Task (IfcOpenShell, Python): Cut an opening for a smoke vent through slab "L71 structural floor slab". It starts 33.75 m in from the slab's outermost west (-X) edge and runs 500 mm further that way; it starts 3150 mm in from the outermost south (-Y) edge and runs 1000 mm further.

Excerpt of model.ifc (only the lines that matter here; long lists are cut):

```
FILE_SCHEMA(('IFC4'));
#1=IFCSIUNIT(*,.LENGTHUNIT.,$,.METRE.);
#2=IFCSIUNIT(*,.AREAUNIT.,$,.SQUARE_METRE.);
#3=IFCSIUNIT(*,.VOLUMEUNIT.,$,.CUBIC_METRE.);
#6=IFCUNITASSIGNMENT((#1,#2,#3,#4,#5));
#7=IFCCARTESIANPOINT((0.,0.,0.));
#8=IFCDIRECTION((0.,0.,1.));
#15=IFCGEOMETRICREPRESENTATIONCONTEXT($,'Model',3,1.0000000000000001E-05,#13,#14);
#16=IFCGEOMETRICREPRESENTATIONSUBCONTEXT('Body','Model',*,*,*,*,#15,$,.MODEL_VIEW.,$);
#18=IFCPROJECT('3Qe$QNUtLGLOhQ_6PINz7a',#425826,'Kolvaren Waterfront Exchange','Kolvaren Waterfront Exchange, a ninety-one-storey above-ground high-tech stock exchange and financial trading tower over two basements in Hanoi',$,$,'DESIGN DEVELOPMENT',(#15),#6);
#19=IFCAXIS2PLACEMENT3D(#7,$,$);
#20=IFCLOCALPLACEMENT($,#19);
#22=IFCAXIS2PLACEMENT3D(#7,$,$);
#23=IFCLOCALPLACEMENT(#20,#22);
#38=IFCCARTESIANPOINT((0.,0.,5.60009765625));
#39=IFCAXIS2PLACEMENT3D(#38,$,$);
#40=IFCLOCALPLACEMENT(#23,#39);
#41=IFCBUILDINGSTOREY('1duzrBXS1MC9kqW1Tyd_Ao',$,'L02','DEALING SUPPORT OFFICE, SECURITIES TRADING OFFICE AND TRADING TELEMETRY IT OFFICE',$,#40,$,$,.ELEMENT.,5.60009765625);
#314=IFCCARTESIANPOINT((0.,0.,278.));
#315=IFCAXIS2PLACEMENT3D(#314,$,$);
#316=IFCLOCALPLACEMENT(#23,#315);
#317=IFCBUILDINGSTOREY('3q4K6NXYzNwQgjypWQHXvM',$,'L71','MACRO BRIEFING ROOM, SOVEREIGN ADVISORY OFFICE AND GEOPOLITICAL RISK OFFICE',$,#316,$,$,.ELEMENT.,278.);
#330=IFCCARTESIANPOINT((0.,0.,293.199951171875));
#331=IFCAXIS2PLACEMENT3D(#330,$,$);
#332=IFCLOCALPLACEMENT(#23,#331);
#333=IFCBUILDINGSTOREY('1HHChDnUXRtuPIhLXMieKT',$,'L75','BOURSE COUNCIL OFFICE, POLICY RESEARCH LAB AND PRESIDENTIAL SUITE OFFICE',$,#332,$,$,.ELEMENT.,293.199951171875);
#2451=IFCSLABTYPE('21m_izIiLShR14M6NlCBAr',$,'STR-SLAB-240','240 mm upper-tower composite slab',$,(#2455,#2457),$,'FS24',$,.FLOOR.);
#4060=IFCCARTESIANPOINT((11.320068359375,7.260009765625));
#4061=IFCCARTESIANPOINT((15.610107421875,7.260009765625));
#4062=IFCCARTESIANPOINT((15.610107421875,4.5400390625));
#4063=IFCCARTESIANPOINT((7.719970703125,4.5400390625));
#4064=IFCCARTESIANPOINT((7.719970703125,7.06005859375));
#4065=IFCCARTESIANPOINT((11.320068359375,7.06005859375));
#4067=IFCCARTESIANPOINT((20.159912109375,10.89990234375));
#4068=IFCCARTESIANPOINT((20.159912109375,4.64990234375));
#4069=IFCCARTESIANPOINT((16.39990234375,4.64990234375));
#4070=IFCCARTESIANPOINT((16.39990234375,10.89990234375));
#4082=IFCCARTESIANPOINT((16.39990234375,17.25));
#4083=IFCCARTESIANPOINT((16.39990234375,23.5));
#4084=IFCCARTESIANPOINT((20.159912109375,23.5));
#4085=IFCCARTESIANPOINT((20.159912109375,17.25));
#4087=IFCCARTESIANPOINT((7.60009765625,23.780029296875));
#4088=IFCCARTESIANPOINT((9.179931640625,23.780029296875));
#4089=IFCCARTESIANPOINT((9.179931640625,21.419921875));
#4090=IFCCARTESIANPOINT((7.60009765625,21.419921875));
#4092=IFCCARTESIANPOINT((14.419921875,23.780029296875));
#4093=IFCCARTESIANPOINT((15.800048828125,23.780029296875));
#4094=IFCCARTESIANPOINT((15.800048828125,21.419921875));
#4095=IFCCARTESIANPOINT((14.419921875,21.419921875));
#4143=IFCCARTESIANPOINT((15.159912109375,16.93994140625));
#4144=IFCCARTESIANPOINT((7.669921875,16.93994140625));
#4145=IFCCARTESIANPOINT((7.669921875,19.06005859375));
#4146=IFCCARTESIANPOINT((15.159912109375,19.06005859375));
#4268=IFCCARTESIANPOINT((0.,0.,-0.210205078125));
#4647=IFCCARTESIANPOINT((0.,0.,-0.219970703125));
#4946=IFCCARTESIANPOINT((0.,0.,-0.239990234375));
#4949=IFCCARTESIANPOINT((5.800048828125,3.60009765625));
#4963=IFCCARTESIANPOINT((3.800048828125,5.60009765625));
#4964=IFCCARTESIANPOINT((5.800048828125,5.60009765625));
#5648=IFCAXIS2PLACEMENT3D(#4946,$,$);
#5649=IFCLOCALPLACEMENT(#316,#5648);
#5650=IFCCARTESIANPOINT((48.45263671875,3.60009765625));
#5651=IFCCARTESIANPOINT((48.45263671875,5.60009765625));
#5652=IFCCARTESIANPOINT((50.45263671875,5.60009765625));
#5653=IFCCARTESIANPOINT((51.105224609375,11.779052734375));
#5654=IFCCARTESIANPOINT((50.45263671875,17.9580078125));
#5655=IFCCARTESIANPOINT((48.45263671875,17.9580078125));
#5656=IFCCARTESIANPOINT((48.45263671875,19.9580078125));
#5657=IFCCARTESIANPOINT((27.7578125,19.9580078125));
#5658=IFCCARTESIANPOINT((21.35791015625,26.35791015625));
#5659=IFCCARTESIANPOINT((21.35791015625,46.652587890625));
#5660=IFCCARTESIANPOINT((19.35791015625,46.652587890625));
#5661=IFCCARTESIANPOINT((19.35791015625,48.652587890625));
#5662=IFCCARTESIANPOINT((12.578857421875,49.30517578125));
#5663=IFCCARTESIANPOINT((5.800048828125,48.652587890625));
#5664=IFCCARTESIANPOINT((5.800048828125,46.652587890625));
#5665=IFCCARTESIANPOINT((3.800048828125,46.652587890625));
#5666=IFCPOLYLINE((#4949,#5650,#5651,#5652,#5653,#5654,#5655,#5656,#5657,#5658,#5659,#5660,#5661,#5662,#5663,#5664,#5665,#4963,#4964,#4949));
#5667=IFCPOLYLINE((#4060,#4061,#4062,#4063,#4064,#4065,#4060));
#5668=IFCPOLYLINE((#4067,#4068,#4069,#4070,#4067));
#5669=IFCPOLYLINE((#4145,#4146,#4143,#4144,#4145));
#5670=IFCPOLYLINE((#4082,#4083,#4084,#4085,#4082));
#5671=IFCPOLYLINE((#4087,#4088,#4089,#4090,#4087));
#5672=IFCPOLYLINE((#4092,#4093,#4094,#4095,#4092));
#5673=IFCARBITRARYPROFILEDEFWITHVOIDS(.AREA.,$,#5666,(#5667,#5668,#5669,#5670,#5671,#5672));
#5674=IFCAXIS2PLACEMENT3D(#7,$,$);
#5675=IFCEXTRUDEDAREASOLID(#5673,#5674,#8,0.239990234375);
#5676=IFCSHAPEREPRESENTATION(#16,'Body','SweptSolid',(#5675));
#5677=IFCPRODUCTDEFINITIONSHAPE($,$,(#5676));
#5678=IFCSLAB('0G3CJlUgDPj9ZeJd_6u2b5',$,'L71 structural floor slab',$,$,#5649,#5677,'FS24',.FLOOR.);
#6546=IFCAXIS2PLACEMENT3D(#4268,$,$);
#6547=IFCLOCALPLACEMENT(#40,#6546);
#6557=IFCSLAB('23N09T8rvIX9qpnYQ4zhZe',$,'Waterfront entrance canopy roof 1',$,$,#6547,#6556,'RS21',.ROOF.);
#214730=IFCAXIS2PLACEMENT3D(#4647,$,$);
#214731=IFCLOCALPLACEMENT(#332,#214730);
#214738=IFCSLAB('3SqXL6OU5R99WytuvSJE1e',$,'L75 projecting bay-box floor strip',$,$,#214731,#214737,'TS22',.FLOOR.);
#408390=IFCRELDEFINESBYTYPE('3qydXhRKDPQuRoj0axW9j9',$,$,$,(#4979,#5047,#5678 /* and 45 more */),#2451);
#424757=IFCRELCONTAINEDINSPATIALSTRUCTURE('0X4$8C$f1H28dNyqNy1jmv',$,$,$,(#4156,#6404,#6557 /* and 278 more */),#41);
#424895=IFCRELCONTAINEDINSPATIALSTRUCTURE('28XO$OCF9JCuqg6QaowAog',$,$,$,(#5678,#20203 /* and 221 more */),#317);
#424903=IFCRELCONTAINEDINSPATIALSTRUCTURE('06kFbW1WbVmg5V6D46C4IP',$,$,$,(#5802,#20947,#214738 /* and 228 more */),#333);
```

```python
import numpy as np
import ifcopenshell
import ifcopenshell.api.feature
import ifcopenshell.api.geometry
import ifcopenshell.api.root
import ifcopenshell.geom
import ifcopenshell.util.placement
import ifcopenshell.util.representation
import ifcopenshell.util.shape
import ifcopenshell.util.unit

model = ifcopenshell.open("model.ifc")
unit_scale = ifcopenshell.util.unit.calculate_unit_scale(model)
settings = ifcopenshell.geom.settings()


def volume(element):
    """Net volume in cubic metres, openings subtracted."""
    shape = ifcopenshell.geom.create_shape(settings, element)
    return ifcopenshell.util.shape.get_volume(shape.geometry)


slab = model.by_guid("0G3CJlUgDPj9ZeJd_6u2b5")
before = volume(slab)

# Extent in the slab's own axes, in metres. The edges named are its -X and -Y sides.
slab_shape = ifcopenshell.geom.create_shape(settings, slab)
vertices = ifcopenshell.util.shape.get_vertices(slab_shape.geometry)
x_min, y_min, bottom = vertices.min(axis=0)
top = vertices[:, 2].max()

opening = ifcopenshell.api.root.create_entity(model, ifc_class="IfcOpeningElement", name="Smoke vent opening", predefined_type="OPENING")
context = ifcopenshell.util.representation.get_context(model, "Model", "Body", "MODEL_VIEW")
width, depth = 0.5, 1
outline = [(0.0, 0.0), (width, 0.0), (width, depth), (0.0, depth), (0.0, 0.0)]
# Overshoot both faces by 50 mm so the cut is clean.
shape = ifcopenshell.api.geometry.add_slab_representation(
    model, context=context, depth=top - bottom + 0.1, polyline=outline
)
ifcopenshell.api.geometry.assign_representation(model, product=opening, representation=shape)

matrix = ifcopenshell.util.placement.get_local_placement(slab.ObjectPlacement)
matrix[:, 3] = matrix @ np.append(np.array([x_min + 33.75, y_min + 3.15, bottom - 0.05]) / unit_scale, 1.0)
ifcopenshell.api.geometry.edit_object_placement(model, product=opening, matrix=matrix, is_si=False)
ifcopenshell.api.feature.add_feature(model, feature=opening, element=slab)

after = volume(slab)

print(f"slab volume {before:.3f} -> {after:.3f} m3")

model.write("model-out.ifc")
```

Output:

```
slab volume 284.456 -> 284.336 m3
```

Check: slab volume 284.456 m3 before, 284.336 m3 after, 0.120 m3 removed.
